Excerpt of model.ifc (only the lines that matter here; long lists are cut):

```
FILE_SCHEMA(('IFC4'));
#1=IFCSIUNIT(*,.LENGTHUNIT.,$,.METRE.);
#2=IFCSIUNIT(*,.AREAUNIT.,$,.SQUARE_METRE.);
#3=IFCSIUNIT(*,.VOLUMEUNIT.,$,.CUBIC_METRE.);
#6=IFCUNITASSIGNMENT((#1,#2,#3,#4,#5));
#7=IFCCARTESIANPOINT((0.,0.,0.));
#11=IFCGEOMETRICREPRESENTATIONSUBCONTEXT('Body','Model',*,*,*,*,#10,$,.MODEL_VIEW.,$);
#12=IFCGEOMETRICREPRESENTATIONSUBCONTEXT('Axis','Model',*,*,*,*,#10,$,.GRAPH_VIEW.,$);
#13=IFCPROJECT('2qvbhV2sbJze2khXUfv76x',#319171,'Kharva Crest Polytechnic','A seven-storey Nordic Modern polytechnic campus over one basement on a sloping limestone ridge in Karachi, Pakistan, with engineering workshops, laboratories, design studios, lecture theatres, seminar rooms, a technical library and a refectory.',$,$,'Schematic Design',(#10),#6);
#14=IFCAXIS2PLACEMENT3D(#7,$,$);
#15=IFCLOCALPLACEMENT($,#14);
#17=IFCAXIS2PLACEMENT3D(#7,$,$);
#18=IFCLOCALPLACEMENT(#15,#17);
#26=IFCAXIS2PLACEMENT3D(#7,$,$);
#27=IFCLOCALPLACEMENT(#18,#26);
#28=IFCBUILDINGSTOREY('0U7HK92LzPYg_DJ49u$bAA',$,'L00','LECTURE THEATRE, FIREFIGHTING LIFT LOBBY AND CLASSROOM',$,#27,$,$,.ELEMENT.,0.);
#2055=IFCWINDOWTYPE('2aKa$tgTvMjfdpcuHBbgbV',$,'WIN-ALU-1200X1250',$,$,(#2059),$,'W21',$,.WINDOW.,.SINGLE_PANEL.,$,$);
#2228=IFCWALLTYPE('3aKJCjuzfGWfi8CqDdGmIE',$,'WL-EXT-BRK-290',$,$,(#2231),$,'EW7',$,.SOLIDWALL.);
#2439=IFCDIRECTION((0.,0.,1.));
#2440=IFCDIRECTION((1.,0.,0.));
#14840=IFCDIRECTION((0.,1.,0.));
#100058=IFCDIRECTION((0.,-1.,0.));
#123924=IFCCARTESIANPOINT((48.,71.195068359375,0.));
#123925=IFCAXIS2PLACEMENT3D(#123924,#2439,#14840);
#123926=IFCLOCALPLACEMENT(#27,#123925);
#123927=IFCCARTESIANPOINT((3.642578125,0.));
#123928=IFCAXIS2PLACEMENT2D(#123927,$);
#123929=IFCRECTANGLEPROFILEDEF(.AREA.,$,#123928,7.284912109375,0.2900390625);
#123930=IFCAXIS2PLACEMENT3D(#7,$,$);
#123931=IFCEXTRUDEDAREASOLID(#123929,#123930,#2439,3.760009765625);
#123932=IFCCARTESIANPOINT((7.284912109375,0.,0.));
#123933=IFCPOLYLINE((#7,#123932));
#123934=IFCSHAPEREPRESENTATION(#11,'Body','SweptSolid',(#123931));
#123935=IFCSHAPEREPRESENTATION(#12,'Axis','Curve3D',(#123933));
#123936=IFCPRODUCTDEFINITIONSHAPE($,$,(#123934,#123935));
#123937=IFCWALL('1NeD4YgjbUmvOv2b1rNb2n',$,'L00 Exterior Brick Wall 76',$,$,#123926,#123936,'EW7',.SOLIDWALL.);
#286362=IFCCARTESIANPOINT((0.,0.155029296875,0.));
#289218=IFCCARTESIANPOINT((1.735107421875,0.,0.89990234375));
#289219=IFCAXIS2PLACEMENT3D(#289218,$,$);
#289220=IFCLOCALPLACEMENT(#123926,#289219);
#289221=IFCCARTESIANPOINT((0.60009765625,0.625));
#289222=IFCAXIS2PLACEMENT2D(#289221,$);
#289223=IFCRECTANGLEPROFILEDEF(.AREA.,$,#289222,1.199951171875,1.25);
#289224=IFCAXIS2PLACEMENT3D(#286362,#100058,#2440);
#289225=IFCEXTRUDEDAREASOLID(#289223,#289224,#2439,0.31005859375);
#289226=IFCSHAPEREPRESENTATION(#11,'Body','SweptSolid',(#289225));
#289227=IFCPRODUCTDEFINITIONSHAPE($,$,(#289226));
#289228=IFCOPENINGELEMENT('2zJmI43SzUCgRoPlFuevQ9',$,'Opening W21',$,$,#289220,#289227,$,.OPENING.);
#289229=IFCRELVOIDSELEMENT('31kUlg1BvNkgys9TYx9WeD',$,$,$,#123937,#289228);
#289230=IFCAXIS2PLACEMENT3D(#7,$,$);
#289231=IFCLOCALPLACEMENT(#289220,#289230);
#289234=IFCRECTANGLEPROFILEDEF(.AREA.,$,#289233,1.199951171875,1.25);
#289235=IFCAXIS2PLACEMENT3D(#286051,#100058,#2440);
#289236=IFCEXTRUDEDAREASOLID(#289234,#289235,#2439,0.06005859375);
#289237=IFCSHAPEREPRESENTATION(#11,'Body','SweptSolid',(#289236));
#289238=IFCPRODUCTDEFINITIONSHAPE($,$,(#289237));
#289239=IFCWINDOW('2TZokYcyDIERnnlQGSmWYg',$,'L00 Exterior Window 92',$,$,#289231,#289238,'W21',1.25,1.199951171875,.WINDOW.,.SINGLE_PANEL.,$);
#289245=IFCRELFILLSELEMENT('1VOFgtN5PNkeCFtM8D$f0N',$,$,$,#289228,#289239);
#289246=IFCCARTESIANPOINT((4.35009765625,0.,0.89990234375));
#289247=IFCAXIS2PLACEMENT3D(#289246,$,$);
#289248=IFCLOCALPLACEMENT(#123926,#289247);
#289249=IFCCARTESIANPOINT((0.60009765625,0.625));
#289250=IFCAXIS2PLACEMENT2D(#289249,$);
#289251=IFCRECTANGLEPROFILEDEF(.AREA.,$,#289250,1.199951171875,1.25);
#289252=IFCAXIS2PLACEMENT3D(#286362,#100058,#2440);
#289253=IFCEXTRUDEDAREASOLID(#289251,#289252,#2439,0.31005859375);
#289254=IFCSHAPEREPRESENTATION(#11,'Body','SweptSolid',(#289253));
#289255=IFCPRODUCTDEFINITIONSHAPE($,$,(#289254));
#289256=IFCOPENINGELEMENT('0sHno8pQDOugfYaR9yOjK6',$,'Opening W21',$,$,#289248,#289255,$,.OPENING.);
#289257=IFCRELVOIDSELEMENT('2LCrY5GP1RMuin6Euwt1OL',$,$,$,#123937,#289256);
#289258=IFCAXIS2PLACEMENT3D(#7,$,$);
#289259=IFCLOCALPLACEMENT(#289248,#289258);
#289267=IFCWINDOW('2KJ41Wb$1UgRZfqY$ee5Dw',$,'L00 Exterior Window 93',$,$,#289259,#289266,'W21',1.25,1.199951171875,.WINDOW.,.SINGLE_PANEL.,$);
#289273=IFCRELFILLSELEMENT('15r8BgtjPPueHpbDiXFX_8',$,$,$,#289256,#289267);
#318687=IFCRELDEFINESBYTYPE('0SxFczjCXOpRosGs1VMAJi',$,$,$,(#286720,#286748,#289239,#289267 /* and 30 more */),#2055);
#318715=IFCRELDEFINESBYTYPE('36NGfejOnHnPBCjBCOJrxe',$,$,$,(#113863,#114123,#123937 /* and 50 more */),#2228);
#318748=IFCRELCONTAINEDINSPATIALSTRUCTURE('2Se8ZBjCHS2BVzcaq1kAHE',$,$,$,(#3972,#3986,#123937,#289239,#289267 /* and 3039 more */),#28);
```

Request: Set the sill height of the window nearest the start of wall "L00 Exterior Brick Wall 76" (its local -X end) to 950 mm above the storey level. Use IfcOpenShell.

```python
import numpy as np
import ifcopenshell
import ifcopenshell.api.geometry
import ifcopenshell.geom
import ifcopenshell.util.element
import ifcopenshell.util.placement
import ifcopenshell.util.shape
import ifcopenshell.util.unit

model = ifcopenshell.open("model.ifc")
unit_scale = ifcopenshell.util.unit.calculate_unit_scale(model)

window = model.by_id(289239)
opening = window.FillsVoids[0].RelatingOpeningElement
storey = ifcopenshell.util.element.get_container(window, ifc_class="IfcBuildingStorey")
level = ifcopenshell.util.placement.get_local_placement(storey.ObjectPlacement)[2, 3]

# The opening's origin need not be at the sill, so measure its lowest point.
shape = ifcopenshell.geom.create_shape(ifcopenshell.geom.settings(), opening)
bottom = ifcopenshell.util.shape.get_shape_bottom_elevation(shape, shape.geometry) / unit_scale
dz = level + 0.95 / unit_scale - bottom

shift = np.array([0.0, 0.0, dz])
# The window is placed relative to its opening, so it follows when the opening moves.
matrix = ifcopenshell.util.placement.get_local_placement(opening.ObjectPlacement)
matrix[:3, 3] += shift
ifcopenshell.api.geometry.edit_object_placement(
    model, product=opening, matrix=matrix, is_si=False, should_transform_children=True
)

print(f"moved by {dz * unit_scale:+.3f} m")

model.write("model_updated.ifc")
```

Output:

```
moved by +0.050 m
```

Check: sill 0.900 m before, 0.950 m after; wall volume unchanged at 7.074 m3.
